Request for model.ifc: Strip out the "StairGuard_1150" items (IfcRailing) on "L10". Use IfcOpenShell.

First a look at what the model holds.

```python
import ifcopenshell
import ifcopenshell.util.element

model = ifcopenshell.open("model.ifc")
print(model.schema)
storey = next(s for s in model.by_type("IfcBuildingStorey") if s.Name == "L10")
railings = [e for e in ifcopenshell.util.element.get_decomposition(storey) if e.is_a("IfcRailing")]
seen = {}
for e in railings:
    element_type = ifcopenshell.util.element.get_type(e)
    name = element_type.Name if element_type not in (None, e) else None
    seen[name] = seen.get(name, 0) + 1
for name, count in sorted(seen.items(), key=str):
    print(count, "x", name)
```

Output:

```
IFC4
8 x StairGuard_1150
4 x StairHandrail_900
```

```python
import ifcopenshell
import ifcopenshell.api.root
import ifcopenshell.util.element

model = ifcopenshell.open("model.ifc")

storey = next(s for s in model.by_type("IfcBuildingStorey") if s.Name == "L10")
railings = [e for e in ifcopenshell.util.element.get_decomposition(storey) if e.is_a("IfcRailing")]
targets = [e for e in railings if (t := ifcopenshell.util.element.get_type(e)) not in (None, e) and t.Name == "StairGuard_1150"]

for e in targets:
    ifcopenshell.api.root.remove_product(model, product=e)
print(len(targets), "removed")

model.write("model-out.ifc")
```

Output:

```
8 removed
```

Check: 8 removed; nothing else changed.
